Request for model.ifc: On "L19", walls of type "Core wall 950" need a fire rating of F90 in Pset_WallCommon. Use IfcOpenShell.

First a look at what the model holds.

```python
import ifcopenshell
import ifcopenshell.util.element

model = ifcopenshell.open("model.ifc")
print(model.schema)
storey = next(s for s in model.by_type("IfcBuildingStorey") if s.Name == "L19")
walls = [e for e in ifcopenshell.util.element.get_decomposition(storey) if e.is_a("IfcWall")]
seen = {}
for e in walls:
    element_type = ifcopenshell.util.element.get_type(e)
    key = (element_type.Name if element_type != e and element_type else None, ifcopenshell.util.element.get_pset(e, "Pset_WallCommon", "FireRating"))
    seen[key] = seen.get(key, 0) + 1
for (name, value), count in sorted(seen.items(), key=str):
    print(count, "x", name, "|", value)
```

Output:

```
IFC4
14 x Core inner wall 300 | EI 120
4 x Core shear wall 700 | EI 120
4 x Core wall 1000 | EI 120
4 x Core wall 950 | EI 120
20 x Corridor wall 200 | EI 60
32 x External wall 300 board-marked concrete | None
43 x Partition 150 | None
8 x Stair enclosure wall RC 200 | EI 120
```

```python
import ifcopenshell
import ifcopenshell.api.pset
import ifcopenshell.util.element

model = ifcopenshell.open("model.ifc")

storey = next(s for s in model.by_type("IfcBuildingStorey") if s.Name == "L19")
walls = [e for e in ifcopenshell.util.element.get_decomposition(storey) if e.is_a("IfcWall")]

count = 0
for e in walls:
    element_type = ifcopenshell.util.element.get_type(e)
    if element_type in (None, e) or element_type.Name != "Core wall 950":
        continue
    # add_pset returns the element's existing set when there is one.
    pset = ifcopenshell.api.pset.add_pset(model, product=e, name="Pset_WallCommon")
    ifcopenshell.api.pset.edit_pset(model, pset=pset, properties={"FireRating": "F90"})
    count += 1

print(count, "walls updated")

model.write("model_v2.ifc")
```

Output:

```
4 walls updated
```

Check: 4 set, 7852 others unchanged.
